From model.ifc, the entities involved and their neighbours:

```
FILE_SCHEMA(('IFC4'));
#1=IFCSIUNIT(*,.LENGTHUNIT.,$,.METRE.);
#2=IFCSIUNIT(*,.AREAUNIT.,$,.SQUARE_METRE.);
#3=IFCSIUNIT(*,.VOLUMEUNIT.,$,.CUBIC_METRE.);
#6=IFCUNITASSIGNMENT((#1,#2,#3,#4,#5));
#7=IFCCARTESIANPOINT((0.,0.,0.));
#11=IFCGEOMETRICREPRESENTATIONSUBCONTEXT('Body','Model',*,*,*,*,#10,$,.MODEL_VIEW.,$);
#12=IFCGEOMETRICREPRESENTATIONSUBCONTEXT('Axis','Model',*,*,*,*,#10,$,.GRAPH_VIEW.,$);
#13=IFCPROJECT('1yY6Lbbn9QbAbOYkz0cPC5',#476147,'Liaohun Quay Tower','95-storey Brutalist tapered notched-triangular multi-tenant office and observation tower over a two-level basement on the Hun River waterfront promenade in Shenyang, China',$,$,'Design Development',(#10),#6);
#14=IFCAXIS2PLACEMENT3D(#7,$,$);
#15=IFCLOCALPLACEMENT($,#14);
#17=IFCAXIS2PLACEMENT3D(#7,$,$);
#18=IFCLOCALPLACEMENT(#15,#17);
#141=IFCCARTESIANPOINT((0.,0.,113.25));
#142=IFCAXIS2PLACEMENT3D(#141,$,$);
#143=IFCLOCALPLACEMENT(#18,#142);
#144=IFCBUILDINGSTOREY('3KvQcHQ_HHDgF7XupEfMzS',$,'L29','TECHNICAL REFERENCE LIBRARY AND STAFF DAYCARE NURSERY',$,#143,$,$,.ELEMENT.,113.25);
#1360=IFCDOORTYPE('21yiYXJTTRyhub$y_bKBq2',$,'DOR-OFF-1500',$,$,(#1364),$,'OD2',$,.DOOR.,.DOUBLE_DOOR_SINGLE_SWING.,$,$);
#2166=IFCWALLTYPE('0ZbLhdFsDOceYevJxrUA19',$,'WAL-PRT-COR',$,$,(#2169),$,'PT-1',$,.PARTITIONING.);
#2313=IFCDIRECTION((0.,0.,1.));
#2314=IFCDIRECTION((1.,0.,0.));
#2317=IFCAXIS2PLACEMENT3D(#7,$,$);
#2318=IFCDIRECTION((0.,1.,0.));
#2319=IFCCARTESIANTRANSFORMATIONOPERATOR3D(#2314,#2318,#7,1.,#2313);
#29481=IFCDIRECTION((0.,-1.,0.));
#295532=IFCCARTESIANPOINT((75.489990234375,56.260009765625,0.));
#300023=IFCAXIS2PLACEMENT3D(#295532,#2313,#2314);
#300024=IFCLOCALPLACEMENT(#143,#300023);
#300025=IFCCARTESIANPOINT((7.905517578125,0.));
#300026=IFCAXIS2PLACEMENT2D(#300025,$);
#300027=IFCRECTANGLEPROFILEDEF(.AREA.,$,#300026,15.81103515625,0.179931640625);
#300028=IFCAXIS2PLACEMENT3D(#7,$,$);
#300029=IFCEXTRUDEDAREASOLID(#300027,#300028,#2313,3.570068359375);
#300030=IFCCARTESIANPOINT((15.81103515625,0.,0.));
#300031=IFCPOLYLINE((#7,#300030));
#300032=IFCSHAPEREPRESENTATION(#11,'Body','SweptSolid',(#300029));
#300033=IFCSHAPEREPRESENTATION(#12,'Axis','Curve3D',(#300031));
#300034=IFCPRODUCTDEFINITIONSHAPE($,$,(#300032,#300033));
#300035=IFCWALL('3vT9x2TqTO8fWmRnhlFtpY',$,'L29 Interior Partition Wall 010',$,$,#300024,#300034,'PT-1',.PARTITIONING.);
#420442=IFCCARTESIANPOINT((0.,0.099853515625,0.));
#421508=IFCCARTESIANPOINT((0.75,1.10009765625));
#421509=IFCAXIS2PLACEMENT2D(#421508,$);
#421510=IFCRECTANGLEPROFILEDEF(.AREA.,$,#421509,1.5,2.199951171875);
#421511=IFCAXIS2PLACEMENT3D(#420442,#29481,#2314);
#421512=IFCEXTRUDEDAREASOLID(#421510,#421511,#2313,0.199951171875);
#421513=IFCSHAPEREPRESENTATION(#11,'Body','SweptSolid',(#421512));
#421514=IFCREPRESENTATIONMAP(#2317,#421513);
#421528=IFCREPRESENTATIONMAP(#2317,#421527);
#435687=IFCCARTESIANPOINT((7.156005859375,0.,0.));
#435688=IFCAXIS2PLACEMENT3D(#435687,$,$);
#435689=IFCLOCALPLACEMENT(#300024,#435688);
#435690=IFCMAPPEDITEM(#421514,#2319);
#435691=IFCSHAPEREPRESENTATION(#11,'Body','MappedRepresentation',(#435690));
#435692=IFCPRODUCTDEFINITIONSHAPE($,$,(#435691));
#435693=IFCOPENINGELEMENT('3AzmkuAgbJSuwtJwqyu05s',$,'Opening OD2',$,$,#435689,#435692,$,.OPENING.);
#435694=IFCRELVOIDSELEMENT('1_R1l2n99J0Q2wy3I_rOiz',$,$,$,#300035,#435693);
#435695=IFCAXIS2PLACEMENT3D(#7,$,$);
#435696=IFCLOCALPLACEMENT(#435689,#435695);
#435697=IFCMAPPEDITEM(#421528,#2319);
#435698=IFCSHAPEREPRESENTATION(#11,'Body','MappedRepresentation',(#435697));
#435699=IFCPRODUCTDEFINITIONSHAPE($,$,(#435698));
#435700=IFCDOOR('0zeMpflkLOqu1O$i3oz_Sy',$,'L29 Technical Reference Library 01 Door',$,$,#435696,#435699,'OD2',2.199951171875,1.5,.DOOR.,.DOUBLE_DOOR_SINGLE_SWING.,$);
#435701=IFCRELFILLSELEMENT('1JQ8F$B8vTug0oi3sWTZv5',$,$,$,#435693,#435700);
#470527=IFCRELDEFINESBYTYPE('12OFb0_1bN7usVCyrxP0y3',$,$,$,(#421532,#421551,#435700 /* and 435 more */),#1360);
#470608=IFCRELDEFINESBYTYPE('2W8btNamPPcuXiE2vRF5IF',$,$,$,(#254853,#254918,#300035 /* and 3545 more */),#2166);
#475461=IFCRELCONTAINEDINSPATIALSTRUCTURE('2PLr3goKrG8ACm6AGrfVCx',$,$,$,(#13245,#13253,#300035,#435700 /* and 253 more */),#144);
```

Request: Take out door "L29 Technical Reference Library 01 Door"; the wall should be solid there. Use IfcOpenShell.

```python
import ifcopenshell
import ifcopenshell.api.feature
import ifcopenshell.api.root
import ifcopenshell.geom
import ifcopenshell.util.shape

model = ifcopenshell.open("model.ifc")
settings = ifcopenshell.geom.settings()


def volume(element):
    """Net volume in cubic metres, openings subtracted."""
    shape = ifcopenshell.geom.create_shape(settings, element)
    return ifcopenshell.util.shape.get_volume(shape.geometry)


door = model.by_guid("0zeMpflkLOqu1O$i3oz_Sy")
opening = door.FillsVoids[0].RelatingOpeningElement
wall = opening.VoidsElements[0].RelatingBuildingElement
before = volume(wall)

ifcopenshell.api.root.remove_product(model, product=door)
ifcopenshell.api.feature.remove_feature(model, feature=opening)

after = volume(wall)

print(f"wall volume {before:.3f} -> {after:.3f} m3")

model.write("model_v2.ifc")
```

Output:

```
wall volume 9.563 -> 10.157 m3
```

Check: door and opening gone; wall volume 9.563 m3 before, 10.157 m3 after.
